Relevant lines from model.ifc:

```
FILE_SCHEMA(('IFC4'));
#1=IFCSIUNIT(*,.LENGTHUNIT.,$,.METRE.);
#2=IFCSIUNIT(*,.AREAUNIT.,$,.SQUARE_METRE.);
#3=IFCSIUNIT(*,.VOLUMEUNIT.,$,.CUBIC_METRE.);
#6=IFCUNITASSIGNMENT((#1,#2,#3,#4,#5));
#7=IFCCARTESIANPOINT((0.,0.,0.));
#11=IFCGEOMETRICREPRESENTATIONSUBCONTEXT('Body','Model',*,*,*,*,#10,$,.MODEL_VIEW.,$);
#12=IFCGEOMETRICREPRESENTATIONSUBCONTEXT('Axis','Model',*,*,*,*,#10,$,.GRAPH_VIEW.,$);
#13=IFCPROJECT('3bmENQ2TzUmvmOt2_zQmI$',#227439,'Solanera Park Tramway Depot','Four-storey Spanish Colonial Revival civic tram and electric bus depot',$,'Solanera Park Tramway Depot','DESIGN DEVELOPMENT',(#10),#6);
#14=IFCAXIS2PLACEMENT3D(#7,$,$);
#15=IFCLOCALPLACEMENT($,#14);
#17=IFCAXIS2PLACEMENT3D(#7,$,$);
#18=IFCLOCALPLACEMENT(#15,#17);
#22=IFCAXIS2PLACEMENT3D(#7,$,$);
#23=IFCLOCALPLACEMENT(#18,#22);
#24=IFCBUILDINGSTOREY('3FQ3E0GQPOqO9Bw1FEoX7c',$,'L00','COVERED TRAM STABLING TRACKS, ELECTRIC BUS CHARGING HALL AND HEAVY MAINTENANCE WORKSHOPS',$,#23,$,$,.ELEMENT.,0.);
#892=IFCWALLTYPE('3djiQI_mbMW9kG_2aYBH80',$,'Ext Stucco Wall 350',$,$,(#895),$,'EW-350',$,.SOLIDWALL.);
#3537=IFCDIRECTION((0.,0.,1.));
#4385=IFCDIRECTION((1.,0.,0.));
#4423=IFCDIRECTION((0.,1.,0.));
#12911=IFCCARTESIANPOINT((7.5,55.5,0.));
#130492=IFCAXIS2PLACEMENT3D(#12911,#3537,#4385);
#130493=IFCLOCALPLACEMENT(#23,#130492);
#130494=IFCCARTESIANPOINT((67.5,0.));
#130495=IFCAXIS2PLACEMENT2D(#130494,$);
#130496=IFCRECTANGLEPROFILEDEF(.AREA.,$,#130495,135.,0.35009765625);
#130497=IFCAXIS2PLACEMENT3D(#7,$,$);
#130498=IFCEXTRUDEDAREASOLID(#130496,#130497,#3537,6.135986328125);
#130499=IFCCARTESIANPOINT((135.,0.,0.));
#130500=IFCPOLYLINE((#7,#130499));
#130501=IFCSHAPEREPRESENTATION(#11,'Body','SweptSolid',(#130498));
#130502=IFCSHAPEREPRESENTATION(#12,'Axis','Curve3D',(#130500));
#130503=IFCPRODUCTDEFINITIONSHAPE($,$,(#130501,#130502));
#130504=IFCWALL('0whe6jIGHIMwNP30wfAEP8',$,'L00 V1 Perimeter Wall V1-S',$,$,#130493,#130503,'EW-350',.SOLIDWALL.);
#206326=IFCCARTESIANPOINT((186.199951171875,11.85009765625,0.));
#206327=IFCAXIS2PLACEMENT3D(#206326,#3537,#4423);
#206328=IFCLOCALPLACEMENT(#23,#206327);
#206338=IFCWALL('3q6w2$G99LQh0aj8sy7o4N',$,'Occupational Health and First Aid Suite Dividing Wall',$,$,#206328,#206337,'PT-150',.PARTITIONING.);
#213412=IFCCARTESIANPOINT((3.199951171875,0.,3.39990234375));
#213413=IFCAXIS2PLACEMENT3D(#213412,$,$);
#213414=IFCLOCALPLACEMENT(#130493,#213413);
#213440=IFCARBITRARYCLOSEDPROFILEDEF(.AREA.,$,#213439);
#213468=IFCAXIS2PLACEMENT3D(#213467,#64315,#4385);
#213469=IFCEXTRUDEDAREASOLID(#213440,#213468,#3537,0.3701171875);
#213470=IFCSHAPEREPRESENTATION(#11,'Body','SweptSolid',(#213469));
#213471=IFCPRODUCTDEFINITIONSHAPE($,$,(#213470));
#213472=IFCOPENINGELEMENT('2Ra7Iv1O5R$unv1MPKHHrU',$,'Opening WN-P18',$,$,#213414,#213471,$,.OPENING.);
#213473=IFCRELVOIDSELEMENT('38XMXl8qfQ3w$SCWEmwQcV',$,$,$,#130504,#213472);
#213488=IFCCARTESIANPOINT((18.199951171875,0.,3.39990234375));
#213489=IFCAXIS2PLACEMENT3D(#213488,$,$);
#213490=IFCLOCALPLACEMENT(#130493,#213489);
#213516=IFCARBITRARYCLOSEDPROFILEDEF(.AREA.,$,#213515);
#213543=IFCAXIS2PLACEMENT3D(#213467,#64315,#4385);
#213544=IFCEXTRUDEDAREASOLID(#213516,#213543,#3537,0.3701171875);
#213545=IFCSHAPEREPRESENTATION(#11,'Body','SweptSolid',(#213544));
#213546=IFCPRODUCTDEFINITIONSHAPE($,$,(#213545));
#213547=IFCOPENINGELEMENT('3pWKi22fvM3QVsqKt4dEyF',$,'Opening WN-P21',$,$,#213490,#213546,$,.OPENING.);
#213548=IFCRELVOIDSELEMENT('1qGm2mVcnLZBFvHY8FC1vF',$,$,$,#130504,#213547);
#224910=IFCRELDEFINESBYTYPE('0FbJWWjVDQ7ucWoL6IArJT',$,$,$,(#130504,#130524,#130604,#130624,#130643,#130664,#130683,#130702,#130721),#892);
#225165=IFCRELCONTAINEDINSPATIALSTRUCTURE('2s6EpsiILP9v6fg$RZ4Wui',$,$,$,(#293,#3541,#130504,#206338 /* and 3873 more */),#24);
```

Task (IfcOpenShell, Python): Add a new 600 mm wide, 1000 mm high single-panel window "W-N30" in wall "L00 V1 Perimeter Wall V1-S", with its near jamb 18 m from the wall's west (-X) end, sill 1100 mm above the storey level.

```python
import numpy as np
import ifcopenshell
import ifcopenshell.api.feature
import ifcopenshell.api.geometry
import ifcopenshell.api.root
import ifcopenshell.api.spatial
import ifcopenshell.geom
import ifcopenshell.util.element
import ifcopenshell.util.placement
import ifcopenshell.util.representation
import ifcopenshell.util.shape
import ifcopenshell.util.unit

model = ifcopenshell.open("model.ifc")
unit_scale = ifcopenshell.util.unit.calculate_unit_scale(model)
settings = ifcopenshell.geom.settings()


def volume(element):
    """Net volume in cubic metres, openings subtracted."""
    shape = ifcopenshell.geom.create_shape(settings, element)
    return ifcopenshell.util.shape.get_volume(shape.geometry)


wall = model.by_guid("0whe6jIGHIMwNP30wfAEP8")
storey = ifcopenshell.util.element.get_container(wall, ifc_class="IfcBuildingStorey")
context = ifcopenshell.util.representation.get_context(model, "Model", "Body", "MODEL_VIEW")
before = volume(wall)

width, height, from_end, sill = 0.6, 1, 18, 1.1  # metres

# The wall runs along its own X axis, and the end named is its -X end.
wall_shape = ifcopenshell.geom.create_shape(settings, wall)
x, y, z = ifcopenshell.util.shape.get_vertices(wall_shape.geometry).T
start = x.min() + from_end
face, thickness = float(y.min()), float(y.max() - y.min())
wall_matrix = ifcopenshell.util.placement.get_local_placement(wall.ObjectPlacement)
level = ifcopenshell.util.placement.get_local_placement(storey.ObjectPlacement)[2, 3]


def in_wall(x, y):
    """Placement at x, y metres in the wall's axes, at sill height."""
    matrix = wall_matrix.copy()
    matrix[:, 3] = wall_matrix @ np.array([x / unit_scale, y / unit_scale, 0.0, 1.0])
    matrix[2, 3] = level + sill / unit_scale
    return matrix


# Opening: a box that overshoots both wall faces by 50 mm.
opening = ifcopenshell.api.root.create_entity(model, ifc_class="IfcOpeningElement", predefined_type="OPENING")
box = ifcopenshell.api.geometry.add_wall_representation(
    model, context=context, length=width, height=height, thickness=thickness + 0.1
)
ifcopenshell.api.geometry.assign_representation(model, product=opening, representation=box)
ifcopenshell.api.geometry.edit_object_placement(model, product=opening, matrix=in_wall(start, face - 0.05), is_si=False)
ifcopenshell.api.feature.add_feature(model, feature=opening, element=wall)

window = ifcopenshell.api.root.create_entity(model, ifc_class="IfcWindow", name="W-N30", predefined_type="WINDOW")
window.OverallWidth, window.OverallHeight = width / unit_scale, height / unit_scale
window.PartitioningType = "SINGLE_PANEL"
body = ifcopenshell.api.geometry.add_window_representation(
    model,
    context=context,
    overall_width=window.OverallWidth,
    overall_height=window.OverallHeight,
    partition_type="SINGLE_PANEL",
)
ifcopenshell.api.geometry.assign_representation(model, product=window, representation=body)
ifcopenshell.api.spatial.assign_container(model, products=[window], relating_structure=storey)
ifcopenshell.api.feature.add_filling(model, opening=opening, element=window)

# Centre the window in the wall's thickness.
ifcopenshell.api.geometry.edit_object_placement(model, product=window, matrix=in_wall(start, face), is_si=False)
window_shape = ifcopenshell.geom.create_shape(settings, window)
depth = ifcopenshell.util.shape.get_vertices(window_shape.geometry)[:, 1]
offset = face + thickness / 2 - (depth.min() + depth.max()) / 2
ifcopenshell.api.geometry.edit_object_placement(model, product=window, matrix=in_wall(start, offset), is_si=False)

after = volume(wall)

print(f"wall volume {before:.3f} -> {after:.3f} m3")

model.write("model_v2.ifc")
```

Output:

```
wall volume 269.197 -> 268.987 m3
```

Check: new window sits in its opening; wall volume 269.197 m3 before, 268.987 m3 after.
